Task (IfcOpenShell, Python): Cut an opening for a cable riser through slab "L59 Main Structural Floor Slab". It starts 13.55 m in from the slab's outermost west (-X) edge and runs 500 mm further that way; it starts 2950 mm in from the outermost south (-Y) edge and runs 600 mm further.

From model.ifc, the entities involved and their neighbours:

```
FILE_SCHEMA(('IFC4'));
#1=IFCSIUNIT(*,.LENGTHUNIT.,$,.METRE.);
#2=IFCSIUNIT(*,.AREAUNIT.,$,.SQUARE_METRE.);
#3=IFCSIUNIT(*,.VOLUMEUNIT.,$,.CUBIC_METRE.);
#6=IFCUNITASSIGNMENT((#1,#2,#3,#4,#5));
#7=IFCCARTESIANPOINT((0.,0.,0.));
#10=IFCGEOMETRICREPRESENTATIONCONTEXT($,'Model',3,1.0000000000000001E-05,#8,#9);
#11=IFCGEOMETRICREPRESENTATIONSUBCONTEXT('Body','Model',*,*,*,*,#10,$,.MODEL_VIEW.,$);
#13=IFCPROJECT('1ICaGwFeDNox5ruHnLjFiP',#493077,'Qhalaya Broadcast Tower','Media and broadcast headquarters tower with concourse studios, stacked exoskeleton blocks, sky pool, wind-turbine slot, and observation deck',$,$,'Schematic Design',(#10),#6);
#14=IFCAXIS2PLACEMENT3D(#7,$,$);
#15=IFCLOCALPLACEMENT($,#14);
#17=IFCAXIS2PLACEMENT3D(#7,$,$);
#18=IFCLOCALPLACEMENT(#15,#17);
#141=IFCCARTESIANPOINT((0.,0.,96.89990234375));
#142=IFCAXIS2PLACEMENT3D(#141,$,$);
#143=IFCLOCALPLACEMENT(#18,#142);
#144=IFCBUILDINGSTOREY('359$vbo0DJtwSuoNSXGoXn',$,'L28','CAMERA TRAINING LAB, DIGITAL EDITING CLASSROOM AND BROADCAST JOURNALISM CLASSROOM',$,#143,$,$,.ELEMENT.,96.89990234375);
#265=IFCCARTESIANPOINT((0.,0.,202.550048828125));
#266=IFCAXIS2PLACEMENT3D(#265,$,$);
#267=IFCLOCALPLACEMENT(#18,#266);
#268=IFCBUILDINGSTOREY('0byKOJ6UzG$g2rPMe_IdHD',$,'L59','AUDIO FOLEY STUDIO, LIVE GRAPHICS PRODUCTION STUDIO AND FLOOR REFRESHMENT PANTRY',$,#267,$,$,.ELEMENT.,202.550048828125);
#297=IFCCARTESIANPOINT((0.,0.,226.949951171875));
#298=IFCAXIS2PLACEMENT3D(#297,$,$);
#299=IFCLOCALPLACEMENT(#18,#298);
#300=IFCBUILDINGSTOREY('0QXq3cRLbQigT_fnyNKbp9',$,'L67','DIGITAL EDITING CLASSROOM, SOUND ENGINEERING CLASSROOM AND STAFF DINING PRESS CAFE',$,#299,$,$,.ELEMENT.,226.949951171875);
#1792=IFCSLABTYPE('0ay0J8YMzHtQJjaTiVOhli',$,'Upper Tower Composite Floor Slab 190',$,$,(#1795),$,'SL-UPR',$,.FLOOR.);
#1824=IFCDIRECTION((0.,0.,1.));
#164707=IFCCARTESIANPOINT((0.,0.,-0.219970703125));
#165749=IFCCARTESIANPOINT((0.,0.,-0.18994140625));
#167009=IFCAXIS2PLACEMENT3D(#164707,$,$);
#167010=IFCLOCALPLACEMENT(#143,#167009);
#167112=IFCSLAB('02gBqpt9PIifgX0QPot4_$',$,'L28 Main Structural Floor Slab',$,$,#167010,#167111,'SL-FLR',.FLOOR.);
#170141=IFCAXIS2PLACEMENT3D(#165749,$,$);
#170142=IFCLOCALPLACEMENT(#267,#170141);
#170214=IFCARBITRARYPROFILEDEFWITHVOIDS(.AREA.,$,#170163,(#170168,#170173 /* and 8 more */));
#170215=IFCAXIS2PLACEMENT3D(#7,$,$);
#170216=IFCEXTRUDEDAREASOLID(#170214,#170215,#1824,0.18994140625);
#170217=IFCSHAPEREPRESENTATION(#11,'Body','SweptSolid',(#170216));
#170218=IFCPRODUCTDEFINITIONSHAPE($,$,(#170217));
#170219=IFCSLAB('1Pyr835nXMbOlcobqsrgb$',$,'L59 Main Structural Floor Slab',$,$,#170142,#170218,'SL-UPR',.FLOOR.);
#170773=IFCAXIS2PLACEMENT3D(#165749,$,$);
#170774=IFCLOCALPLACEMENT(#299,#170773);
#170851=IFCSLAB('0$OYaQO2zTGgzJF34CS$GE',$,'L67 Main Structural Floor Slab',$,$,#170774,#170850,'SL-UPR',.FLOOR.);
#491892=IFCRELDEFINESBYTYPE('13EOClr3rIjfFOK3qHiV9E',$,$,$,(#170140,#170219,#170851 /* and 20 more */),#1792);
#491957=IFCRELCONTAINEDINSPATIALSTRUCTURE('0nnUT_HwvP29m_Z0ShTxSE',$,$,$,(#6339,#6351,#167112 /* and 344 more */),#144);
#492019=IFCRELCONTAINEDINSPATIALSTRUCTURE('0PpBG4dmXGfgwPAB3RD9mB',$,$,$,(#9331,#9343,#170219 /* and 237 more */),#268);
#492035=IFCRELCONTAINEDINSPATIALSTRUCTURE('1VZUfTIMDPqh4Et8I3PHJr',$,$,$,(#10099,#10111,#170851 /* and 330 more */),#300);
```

```python
import numpy as np
import ifcopenshell
import ifcopenshell.api.feature
import ifcopenshell.api.geometry
import ifcopenshell.api.root
import ifcopenshell.geom
import ifcopenshell.util.placement
import ifcopenshell.util.representation
import ifcopenshell.util.shape
import ifcopenshell.util.unit

model = ifcopenshell.open("model.ifc")
unit_scale = ifcopenshell.util.unit.calculate_unit_scale(model)
settings = ifcopenshell.geom.settings()


def volume(element):
    """Net volume in cubic metres, openings subtracted."""
    shape = ifcopenshell.geom.create_shape(settings, element)
    return ifcopenshell.util.shape.get_volume(shape.geometry)


slab = model.by_guid("1Pyr835nXMbOlcobqsrgb$")
before = volume(slab)

# Extent in the slab's own axes, in metres. The edges named are its -X and -Y sides.
slab_shape = ifcopenshell.geom.create_shape(settings, slab)
vertices = ifcopenshell.util.shape.get_vertices(slab_shape.geometry)
x_min, y_min, bottom = vertices.min(axis=0)
top = vertices[:, 2].max()

opening = ifcopenshell.api.root.create_entity(model, ifc_class="IfcOpeningElement", name="Cable riser opening", predefined_type="OPENING")
context = ifcopenshell.util.representation.get_context(model, "Model", "Body", "MODEL_VIEW")
width, depth = 0.5, 0.6
outline = [(0.0, 0.0), (width, 0.0), (width, depth), (0.0, depth), (0.0, 0.0)]
# Overshoot both faces by 50 mm so the cut is clean.
shape = ifcopenshell.api.geometry.add_slab_representation(
    model, context=context, depth=top - bottom + 0.1, polyline=outline
)
ifcopenshell.api.geometry.assign_representation(model, product=opening, representation=shape)

matrix = ifcopenshell.util.placement.get_local_placement(slab.ObjectPlacement)
matrix[:, 3] = matrix @ np.append(np.array([x_min + 13.55, y_min + 2.95, bottom - 0.05]) / unit_scale, 1.0)
ifcopenshell.api.geometry.edit_object_placement(model, product=opening, matrix=matrix, is_si=False)
ifcopenshell.api.feature.add_feature(model, feature=opening, element=slab)

after = volume(slab)

print(f"slab volume {before:.3f} -> {after:.3f} m3")

model.write("model_v2.ifc")
```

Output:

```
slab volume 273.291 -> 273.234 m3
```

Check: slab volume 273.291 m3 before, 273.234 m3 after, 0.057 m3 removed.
